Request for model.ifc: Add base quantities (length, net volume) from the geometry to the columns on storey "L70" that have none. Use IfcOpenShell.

First a look at what the model holds.

```python
import ifcopenshell
import ifcopenshell.util.element
import ifcopenshell.util.unit

model = ifcopenshell.open("model.ifc")
print(model.schema)
for unit_type in ("LENGTHUNIT", "AREAUNIT", "VOLUMEUNIT"):
    print(unit_type, ifcopenshell.util.unit.calculate_unit_scale(model, unit_type))
storey = next(s for s in model.by_type("IfcBuildingStorey") if s.Name == "L70")
columns = [e for e in ifcopenshell.util.element.get_decomposition(storey) if e.is_a("IfcColumn")]
for e in sorted(columns, key=lambda e: e.id()):
    print(e.id(), e.is_a(), e.Name, list(ifcopenshell.util.element.get_psets(e, qtos_only=True)), sep=" | ")
```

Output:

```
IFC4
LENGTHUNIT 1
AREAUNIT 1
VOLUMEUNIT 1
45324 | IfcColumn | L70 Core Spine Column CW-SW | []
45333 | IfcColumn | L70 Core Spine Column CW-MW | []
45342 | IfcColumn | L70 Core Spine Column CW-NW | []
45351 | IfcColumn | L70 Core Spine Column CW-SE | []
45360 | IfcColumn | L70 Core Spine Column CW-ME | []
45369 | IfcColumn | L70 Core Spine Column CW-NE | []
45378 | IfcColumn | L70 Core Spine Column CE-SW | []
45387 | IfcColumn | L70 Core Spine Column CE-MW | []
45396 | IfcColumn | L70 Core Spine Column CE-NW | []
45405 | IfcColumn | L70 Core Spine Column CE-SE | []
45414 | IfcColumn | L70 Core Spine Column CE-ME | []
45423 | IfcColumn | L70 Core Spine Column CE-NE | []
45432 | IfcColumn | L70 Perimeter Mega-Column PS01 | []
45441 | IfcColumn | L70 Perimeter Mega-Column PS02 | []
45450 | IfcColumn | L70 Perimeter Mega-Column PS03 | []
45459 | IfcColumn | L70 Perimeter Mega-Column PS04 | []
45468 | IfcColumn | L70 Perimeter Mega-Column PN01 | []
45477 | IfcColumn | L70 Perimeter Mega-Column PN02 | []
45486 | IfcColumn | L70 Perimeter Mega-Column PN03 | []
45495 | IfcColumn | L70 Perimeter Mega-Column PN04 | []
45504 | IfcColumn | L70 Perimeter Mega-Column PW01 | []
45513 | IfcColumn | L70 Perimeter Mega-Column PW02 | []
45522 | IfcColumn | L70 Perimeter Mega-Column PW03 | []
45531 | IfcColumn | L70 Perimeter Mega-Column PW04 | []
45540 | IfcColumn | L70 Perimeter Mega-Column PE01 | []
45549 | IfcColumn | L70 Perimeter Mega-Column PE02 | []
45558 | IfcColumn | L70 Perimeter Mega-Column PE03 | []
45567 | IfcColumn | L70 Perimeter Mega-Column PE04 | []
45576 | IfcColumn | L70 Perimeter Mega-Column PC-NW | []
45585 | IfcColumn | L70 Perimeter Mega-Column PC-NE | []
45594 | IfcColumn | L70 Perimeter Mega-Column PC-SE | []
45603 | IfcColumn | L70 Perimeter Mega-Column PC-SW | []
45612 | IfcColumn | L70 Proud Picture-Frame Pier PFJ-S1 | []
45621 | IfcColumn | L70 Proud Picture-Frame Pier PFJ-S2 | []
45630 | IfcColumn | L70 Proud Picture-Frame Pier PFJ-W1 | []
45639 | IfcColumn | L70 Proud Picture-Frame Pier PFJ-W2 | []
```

```python
import ifcopenshell
import ifcopenshell.api.pset
import ifcopenshell.geom
import ifcopenshell.util.element
import ifcopenshell.util.shape
import ifcopenshell.util.unit

model = ifcopenshell.open("model.ifc")
unit_scale = ifcopenshell.util.unit.calculate_unit_scale(model)
volume_scale = ifcopenshell.util.unit.calculate_unit_scale(model, "VOLUMEUNIT")
settings = ifcopenshell.geom.settings()

storey = next(s for s in model.by_type("IfcBuildingStorey") if s.Name == "L70")
columns = [e for e in ifcopenshell.util.element.get_decomposition(storey) if e.is_a("IfcColumn")]

for e in sorted(columns, key=lambda e: e.id()):
    if ifcopenshell.util.element.get_psets(e, qtos_only=True, should_inherit=False):
        continue
    # Geometry comes back in metres, in the element's own axes.
    shape = ifcopenshell.geom.create_shape(settings, e)
    values = {
        "Length": ifcopenshell.util.shape.get_z(shape.geometry) / unit_scale,
        "NetVolume": ifcopenshell.util.shape.get_volume(shape.geometry) / volume_scale,
    }
    qto = ifcopenshell.api.pset.add_qto(model, product=e, name="Qto_ColumnBaseQuantities")
    ifcopenshell.api.pset.edit_qto(model, qto=qto, properties=values)
    print(e.id(), {k: round(v, 3) for k, v in values.items()})

model.write("model-out.ifc")
```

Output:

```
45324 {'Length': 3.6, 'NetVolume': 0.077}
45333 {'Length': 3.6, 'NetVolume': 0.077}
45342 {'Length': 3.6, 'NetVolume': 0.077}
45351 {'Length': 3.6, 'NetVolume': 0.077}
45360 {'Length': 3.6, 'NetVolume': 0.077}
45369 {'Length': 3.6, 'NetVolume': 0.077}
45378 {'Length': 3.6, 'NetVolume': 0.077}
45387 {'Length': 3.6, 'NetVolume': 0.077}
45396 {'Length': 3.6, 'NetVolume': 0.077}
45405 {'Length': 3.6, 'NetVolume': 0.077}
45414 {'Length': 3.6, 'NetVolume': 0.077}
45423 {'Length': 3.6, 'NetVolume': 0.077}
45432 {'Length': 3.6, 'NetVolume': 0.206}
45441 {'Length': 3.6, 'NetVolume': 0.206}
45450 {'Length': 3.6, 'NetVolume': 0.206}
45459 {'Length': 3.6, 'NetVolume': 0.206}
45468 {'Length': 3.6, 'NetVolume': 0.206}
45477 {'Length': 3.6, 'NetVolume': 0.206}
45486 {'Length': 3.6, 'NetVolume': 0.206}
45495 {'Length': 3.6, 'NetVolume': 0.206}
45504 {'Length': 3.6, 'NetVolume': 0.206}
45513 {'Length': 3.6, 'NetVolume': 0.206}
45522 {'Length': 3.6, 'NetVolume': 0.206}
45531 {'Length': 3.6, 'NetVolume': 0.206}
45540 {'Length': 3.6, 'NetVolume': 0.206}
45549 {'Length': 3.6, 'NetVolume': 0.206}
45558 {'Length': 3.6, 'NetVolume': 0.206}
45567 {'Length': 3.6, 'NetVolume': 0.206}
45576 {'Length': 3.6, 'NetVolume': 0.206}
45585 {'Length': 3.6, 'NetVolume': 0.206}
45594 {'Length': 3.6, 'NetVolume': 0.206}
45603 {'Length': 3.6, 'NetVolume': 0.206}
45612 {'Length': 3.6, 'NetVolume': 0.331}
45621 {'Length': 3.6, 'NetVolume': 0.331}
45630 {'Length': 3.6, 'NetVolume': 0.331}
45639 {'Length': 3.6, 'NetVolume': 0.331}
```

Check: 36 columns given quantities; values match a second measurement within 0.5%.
